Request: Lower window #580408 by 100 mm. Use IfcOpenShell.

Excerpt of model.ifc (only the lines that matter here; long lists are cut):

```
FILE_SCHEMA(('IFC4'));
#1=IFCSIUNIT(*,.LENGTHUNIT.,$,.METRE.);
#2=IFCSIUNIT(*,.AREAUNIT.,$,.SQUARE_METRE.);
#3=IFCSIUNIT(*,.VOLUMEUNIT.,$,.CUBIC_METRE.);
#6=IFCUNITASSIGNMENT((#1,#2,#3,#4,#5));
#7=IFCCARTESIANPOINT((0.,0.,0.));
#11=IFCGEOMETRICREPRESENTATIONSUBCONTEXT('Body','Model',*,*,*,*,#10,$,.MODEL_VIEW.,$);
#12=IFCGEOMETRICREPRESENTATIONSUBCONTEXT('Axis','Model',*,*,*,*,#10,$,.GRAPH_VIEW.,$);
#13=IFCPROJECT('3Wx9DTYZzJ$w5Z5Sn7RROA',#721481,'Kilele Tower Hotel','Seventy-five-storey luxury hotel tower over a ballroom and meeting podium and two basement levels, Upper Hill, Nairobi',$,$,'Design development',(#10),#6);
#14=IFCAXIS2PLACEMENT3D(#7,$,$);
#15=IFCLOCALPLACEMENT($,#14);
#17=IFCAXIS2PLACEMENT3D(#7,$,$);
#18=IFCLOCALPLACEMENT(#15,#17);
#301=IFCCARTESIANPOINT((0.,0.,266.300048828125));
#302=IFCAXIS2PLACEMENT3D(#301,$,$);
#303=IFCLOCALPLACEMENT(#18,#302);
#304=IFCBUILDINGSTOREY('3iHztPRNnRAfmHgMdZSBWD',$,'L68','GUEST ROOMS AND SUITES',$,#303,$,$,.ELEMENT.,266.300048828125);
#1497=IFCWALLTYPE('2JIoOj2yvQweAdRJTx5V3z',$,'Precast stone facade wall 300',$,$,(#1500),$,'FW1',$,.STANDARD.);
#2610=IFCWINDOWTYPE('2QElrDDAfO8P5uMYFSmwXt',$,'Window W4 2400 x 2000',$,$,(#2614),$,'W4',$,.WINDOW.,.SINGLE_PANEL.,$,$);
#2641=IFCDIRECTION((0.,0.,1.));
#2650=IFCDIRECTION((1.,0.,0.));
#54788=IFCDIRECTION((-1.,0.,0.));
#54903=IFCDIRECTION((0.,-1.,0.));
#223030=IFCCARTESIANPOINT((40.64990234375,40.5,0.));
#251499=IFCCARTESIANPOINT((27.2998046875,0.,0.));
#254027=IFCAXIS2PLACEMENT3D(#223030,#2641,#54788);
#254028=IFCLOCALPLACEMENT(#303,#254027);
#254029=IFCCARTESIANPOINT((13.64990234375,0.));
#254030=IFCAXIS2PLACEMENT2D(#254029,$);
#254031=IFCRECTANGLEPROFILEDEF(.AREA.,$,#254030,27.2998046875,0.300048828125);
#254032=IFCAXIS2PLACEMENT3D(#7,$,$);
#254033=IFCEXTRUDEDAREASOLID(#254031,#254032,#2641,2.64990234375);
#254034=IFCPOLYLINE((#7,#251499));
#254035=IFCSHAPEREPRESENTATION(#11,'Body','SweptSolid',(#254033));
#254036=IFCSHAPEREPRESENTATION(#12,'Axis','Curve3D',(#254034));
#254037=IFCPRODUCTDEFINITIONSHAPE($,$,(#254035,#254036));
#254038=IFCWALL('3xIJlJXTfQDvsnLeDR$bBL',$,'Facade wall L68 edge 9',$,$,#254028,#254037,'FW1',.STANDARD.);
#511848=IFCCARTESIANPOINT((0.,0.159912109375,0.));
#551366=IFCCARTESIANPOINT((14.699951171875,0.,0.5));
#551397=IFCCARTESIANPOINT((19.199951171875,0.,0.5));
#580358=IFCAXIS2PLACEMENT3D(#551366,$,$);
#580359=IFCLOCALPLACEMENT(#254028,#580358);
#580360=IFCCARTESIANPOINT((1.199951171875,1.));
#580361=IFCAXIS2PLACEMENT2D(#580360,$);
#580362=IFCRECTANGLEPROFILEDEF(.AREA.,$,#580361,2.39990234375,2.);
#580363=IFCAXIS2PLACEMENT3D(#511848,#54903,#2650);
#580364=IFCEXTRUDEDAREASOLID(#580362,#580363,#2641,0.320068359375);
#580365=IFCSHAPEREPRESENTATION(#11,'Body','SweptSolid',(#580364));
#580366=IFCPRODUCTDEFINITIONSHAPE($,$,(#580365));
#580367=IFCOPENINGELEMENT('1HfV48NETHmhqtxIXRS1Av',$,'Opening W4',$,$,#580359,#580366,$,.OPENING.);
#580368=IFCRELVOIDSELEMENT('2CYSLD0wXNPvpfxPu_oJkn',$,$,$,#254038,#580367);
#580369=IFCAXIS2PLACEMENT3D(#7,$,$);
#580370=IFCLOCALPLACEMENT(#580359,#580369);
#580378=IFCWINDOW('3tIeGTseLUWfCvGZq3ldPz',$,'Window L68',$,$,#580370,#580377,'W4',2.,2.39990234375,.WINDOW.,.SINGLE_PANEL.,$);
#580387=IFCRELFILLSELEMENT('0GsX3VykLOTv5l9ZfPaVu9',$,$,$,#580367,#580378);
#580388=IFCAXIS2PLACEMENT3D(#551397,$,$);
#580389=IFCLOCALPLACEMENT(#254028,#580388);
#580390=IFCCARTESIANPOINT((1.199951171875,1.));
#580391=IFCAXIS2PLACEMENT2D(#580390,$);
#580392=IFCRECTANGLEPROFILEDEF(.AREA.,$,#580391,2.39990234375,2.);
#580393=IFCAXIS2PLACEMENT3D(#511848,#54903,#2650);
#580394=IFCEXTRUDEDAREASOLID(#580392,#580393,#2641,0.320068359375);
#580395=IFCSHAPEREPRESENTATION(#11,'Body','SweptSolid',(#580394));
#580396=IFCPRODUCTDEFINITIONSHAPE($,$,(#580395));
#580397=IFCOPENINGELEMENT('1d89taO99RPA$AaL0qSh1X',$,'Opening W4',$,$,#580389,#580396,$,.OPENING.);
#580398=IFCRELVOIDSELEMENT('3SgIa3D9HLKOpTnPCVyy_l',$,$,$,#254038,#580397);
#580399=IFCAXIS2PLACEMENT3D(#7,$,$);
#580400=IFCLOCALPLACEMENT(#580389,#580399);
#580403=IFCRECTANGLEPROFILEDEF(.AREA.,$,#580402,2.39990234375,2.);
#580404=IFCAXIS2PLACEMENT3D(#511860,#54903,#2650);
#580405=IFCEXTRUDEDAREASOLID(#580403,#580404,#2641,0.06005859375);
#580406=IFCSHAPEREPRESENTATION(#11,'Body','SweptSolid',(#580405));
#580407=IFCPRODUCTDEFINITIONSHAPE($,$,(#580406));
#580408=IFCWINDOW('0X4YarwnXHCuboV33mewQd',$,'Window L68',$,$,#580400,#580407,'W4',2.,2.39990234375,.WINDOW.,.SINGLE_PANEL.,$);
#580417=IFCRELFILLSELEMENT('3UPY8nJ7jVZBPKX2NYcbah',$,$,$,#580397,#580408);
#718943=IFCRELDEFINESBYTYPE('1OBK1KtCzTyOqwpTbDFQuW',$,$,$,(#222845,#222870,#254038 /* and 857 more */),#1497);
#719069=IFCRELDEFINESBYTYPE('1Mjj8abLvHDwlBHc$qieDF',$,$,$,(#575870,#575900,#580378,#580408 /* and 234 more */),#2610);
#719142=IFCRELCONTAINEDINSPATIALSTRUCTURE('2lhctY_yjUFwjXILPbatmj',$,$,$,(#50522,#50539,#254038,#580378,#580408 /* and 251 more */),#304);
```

```python
import numpy as np
import ifcopenshell
import ifcopenshell.api.geometry
import ifcopenshell.util.placement
import ifcopenshell.util.unit

model = ifcopenshell.open("model.ifc")
unit_scale = ifcopenshell.util.unit.calculate_unit_scale(model)

window = model.by_guid("0X4YarwnXHCuboV33mewQd")
opening = window.FillsVoids[0].RelatingOpeningElement
dz = -0.1 / unit_scale

shift = np.array([0.0, 0.0, dz])
# The window is placed relative to its opening, so it follows when the opening moves.
matrix = ifcopenshell.util.placement.get_local_placement(opening.ObjectPlacement)
matrix[:3, 3] += shift
ifcopenshell.api.geometry.edit_object_placement(
    model, product=opening, matrix=matrix, is_si=False, should_transform_children=True
)

print(f"moved by {dz * unit_scale:+.3f} m")

model.write("model_edited.ifc")
```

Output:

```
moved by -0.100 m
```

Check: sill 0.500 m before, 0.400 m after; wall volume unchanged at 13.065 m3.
